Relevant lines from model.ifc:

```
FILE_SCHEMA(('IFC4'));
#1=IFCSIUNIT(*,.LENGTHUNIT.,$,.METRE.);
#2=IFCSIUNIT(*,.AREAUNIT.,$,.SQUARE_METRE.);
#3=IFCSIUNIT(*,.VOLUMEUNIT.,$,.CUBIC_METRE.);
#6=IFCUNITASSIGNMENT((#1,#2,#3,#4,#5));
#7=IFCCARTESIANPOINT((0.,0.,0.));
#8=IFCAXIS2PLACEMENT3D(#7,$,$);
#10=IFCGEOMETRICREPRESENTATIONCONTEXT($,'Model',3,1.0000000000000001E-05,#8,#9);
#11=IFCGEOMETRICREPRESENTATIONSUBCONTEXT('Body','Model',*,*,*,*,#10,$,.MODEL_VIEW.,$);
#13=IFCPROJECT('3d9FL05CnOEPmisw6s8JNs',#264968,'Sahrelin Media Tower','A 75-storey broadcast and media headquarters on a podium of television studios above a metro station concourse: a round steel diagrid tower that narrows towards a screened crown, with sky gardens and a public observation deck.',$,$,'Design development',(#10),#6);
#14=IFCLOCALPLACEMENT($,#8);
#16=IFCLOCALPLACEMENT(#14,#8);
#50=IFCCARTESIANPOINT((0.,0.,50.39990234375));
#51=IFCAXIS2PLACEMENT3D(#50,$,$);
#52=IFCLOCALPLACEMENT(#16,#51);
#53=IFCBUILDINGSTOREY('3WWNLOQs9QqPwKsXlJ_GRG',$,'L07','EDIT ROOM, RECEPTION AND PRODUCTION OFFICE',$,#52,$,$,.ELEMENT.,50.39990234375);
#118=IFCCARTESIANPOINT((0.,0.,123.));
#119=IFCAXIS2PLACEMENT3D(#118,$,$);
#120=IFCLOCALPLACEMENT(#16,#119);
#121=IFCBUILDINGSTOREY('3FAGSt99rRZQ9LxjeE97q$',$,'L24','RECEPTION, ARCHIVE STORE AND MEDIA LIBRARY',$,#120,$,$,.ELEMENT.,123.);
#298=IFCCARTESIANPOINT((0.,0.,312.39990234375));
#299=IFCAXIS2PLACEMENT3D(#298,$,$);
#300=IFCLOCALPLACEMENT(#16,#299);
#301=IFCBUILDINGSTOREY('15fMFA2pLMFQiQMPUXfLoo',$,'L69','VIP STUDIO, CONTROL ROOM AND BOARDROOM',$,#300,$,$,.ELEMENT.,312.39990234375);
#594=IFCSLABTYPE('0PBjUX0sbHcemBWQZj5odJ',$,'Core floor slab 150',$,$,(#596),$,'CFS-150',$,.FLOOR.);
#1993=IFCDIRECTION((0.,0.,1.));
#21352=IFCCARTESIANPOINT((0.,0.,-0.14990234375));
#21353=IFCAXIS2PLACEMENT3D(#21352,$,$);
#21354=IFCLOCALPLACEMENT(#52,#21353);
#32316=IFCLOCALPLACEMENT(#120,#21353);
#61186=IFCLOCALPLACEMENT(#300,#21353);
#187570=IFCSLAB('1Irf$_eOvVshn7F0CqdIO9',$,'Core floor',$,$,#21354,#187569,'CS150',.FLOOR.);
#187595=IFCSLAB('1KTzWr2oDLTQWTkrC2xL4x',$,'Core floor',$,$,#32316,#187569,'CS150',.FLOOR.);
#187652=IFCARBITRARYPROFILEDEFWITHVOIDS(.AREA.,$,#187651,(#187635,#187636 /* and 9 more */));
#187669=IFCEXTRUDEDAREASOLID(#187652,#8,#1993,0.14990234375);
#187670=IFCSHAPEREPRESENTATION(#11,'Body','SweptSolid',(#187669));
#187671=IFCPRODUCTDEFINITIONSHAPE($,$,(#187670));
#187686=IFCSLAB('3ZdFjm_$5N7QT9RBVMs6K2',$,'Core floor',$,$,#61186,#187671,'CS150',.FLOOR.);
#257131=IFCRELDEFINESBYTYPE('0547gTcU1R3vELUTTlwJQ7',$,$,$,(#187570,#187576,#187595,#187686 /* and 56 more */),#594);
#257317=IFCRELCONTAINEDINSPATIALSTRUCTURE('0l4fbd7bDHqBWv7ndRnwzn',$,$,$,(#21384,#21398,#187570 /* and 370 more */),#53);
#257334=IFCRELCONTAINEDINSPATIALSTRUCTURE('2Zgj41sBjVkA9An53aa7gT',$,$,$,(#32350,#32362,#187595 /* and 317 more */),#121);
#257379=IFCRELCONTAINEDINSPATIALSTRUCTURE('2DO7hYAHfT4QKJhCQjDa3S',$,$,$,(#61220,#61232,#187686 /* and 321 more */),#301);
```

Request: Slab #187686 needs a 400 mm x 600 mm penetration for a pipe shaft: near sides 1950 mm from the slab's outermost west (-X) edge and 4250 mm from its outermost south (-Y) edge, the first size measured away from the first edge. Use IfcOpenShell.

```python
import numpy as np
import ifcopenshell
import ifcopenshell.api.feature
import ifcopenshell.api.geometry
import ifcopenshell.api.root
import ifcopenshell.geom
import ifcopenshell.util.placement
import ifcopenshell.util.representation
import ifcopenshell.util.shape
import ifcopenshell.util.unit

model = ifcopenshell.open("model.ifc")
unit_scale = ifcopenshell.util.unit.calculate_unit_scale(model)
settings = ifcopenshell.geom.settings()


def volume(element):
    """Net volume in cubic metres, openings subtracted."""
    shape = ifcopenshell.geom.create_shape(settings, element)
    return ifcopenshell.util.shape.get_volume(shape.geometry)


slab = model.by_id(187686)
before = volume(slab)

# Extent in the slab's own axes, in metres. The edges named are its -X and -Y sides.
slab_shape = ifcopenshell.geom.create_shape(settings, slab)
vertices = ifcopenshell.util.shape.get_vertices(slab_shape.geometry)
x_min, y_min, bottom = vertices.min(axis=0)
top = vertices[:, 2].max()

opening = ifcopenshell.api.root.create_entity(model, ifc_class="IfcOpeningElement", name="Pipe shaft opening", predefined_type="OPENING")
context = ifcopenshell.util.representation.get_context(model, "Model", "Body", "MODEL_VIEW")
width, depth = 0.4, 0.6
outline = [(0.0, 0.0), (width, 0.0), (width, depth), (0.0, depth), (0.0, 0.0)]
# Overshoot both faces by 50 mm so the cut is clean.
shape = ifcopenshell.api.geometry.add_slab_representation(
    model, context=context, depth=top - bottom + 0.1, polyline=outline
)
ifcopenshell.api.geometry.assign_representation(model, product=opening, representation=shape)

matrix = ifcopenshell.util.placement.get_local_placement(slab.ObjectPlacement)
matrix[:, 3] = matrix @ np.append(np.array([x_min + 1.95, y_min + 4.25, bottom - 0.05]) / unit_scale, 1.0)
ifcopenshell.api.geometry.edit_object_placement(model, product=opening, matrix=matrix, is_si=False)
ifcopenshell.api.feature.add_feature(model, feature=opening, element=slab)

after = volume(slab)

print(f"slab volume {before:.3f} -> {after:.3f} m3")

model.write("model-out.ifc")
```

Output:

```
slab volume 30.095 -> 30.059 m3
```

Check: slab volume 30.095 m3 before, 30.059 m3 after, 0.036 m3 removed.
